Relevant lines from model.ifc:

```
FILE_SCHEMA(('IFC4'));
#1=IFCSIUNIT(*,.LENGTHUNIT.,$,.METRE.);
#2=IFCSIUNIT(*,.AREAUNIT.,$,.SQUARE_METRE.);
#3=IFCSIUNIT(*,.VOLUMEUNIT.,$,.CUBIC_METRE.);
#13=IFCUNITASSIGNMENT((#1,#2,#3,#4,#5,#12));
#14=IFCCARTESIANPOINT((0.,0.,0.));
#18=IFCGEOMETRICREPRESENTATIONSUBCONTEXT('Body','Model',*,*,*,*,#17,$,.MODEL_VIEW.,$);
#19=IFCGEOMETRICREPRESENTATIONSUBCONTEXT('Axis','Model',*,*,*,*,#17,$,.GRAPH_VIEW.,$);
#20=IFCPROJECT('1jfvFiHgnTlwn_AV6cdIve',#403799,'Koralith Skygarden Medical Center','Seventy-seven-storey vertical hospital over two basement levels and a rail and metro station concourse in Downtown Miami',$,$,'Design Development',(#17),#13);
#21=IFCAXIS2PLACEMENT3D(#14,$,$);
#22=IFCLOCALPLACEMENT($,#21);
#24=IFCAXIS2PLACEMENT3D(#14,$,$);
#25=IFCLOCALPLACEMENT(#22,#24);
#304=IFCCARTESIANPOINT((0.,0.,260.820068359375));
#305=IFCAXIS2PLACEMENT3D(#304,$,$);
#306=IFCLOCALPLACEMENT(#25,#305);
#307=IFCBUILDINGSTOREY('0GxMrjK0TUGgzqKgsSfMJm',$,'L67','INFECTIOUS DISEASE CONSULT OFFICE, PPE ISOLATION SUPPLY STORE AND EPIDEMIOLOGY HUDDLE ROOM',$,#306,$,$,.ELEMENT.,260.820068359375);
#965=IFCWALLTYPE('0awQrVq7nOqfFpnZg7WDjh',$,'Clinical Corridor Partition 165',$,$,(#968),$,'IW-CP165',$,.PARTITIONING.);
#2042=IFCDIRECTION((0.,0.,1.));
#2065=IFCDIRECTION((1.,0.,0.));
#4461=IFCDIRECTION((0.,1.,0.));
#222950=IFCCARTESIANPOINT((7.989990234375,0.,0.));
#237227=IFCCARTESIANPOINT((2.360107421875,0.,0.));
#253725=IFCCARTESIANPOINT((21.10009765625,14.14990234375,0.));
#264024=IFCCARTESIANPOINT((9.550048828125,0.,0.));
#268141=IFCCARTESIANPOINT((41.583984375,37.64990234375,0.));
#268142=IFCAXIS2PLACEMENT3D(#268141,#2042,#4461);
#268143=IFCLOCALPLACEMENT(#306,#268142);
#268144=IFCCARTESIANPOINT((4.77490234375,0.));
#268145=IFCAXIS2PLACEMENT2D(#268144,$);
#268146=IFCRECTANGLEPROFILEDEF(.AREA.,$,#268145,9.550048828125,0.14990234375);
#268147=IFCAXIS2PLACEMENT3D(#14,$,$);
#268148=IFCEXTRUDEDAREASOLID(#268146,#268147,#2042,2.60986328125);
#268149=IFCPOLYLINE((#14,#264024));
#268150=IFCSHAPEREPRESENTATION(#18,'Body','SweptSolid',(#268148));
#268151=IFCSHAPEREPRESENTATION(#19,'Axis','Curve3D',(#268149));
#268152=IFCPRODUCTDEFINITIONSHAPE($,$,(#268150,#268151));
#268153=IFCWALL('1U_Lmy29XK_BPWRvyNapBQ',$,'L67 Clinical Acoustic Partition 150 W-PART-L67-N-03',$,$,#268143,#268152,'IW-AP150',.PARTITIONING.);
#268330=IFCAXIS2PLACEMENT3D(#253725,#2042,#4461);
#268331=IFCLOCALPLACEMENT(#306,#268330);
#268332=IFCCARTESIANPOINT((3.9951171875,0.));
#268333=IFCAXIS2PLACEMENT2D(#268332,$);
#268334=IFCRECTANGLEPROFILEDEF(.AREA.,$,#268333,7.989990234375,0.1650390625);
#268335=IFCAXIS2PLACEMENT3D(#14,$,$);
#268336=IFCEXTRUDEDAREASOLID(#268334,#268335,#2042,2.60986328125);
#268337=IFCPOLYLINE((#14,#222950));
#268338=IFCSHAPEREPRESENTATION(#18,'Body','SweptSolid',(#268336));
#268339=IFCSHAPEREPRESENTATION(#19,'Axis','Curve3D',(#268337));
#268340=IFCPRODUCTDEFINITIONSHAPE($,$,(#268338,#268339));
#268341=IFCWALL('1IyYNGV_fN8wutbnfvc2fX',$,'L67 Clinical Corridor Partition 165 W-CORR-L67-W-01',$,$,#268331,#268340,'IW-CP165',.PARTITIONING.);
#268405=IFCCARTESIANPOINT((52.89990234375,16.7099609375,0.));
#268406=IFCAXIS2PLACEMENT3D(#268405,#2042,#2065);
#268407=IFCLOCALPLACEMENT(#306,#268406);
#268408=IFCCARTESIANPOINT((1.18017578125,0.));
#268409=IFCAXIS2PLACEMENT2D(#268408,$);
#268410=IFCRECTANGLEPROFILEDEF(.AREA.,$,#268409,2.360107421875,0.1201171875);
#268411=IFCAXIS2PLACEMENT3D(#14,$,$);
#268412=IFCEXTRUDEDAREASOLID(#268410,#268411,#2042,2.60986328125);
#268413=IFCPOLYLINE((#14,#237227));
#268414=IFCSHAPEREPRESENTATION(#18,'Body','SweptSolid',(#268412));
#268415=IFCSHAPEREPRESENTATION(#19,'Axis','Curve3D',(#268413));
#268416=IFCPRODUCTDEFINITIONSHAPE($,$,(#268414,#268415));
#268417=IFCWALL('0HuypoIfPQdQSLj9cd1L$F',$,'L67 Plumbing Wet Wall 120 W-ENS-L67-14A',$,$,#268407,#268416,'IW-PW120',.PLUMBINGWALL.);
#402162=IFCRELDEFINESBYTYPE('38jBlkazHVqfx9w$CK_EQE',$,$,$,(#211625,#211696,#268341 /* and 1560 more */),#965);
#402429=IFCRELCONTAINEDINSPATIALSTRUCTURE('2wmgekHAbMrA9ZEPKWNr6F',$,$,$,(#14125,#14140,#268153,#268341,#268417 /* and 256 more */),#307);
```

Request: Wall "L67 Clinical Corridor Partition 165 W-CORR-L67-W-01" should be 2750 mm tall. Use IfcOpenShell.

```python
import ifcopenshell
import ifcopenshell.geom
import ifcopenshell.util.representation
import ifcopenshell.util.shape
import ifcopenshell.util.unit

model = ifcopenshell.open("model.ifc")
unit_scale = ifcopenshell.util.unit.calculate_unit_scale(model)
settings = ifcopenshell.geom.settings()


def volume(element):
    """Net volume in cubic metres, openings subtracted."""
    shape = ifcopenshell.geom.create_shape(settings, element)
    return ifcopenshell.util.shape.get_volume(shape.geometry)


wall = model.by_guid("1IyYNGV_fN8wutbnfvc2fX")
before = volume(wall)

body = ifcopenshell.util.representation.get_representation(wall, "Model", "Body")
solid = body.Items[0]
old_height = solid.Depth
solid.Depth = 2.75 / unit_scale
after = volume(wall)

print(f"height {old_height:g} -> {solid.Depth:g}, volume {before:.3f} -> {after:.3f} m3")

model.write("model_rev.ifc")
```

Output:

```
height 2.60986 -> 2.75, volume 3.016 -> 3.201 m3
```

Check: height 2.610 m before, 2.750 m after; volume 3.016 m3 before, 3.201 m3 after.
